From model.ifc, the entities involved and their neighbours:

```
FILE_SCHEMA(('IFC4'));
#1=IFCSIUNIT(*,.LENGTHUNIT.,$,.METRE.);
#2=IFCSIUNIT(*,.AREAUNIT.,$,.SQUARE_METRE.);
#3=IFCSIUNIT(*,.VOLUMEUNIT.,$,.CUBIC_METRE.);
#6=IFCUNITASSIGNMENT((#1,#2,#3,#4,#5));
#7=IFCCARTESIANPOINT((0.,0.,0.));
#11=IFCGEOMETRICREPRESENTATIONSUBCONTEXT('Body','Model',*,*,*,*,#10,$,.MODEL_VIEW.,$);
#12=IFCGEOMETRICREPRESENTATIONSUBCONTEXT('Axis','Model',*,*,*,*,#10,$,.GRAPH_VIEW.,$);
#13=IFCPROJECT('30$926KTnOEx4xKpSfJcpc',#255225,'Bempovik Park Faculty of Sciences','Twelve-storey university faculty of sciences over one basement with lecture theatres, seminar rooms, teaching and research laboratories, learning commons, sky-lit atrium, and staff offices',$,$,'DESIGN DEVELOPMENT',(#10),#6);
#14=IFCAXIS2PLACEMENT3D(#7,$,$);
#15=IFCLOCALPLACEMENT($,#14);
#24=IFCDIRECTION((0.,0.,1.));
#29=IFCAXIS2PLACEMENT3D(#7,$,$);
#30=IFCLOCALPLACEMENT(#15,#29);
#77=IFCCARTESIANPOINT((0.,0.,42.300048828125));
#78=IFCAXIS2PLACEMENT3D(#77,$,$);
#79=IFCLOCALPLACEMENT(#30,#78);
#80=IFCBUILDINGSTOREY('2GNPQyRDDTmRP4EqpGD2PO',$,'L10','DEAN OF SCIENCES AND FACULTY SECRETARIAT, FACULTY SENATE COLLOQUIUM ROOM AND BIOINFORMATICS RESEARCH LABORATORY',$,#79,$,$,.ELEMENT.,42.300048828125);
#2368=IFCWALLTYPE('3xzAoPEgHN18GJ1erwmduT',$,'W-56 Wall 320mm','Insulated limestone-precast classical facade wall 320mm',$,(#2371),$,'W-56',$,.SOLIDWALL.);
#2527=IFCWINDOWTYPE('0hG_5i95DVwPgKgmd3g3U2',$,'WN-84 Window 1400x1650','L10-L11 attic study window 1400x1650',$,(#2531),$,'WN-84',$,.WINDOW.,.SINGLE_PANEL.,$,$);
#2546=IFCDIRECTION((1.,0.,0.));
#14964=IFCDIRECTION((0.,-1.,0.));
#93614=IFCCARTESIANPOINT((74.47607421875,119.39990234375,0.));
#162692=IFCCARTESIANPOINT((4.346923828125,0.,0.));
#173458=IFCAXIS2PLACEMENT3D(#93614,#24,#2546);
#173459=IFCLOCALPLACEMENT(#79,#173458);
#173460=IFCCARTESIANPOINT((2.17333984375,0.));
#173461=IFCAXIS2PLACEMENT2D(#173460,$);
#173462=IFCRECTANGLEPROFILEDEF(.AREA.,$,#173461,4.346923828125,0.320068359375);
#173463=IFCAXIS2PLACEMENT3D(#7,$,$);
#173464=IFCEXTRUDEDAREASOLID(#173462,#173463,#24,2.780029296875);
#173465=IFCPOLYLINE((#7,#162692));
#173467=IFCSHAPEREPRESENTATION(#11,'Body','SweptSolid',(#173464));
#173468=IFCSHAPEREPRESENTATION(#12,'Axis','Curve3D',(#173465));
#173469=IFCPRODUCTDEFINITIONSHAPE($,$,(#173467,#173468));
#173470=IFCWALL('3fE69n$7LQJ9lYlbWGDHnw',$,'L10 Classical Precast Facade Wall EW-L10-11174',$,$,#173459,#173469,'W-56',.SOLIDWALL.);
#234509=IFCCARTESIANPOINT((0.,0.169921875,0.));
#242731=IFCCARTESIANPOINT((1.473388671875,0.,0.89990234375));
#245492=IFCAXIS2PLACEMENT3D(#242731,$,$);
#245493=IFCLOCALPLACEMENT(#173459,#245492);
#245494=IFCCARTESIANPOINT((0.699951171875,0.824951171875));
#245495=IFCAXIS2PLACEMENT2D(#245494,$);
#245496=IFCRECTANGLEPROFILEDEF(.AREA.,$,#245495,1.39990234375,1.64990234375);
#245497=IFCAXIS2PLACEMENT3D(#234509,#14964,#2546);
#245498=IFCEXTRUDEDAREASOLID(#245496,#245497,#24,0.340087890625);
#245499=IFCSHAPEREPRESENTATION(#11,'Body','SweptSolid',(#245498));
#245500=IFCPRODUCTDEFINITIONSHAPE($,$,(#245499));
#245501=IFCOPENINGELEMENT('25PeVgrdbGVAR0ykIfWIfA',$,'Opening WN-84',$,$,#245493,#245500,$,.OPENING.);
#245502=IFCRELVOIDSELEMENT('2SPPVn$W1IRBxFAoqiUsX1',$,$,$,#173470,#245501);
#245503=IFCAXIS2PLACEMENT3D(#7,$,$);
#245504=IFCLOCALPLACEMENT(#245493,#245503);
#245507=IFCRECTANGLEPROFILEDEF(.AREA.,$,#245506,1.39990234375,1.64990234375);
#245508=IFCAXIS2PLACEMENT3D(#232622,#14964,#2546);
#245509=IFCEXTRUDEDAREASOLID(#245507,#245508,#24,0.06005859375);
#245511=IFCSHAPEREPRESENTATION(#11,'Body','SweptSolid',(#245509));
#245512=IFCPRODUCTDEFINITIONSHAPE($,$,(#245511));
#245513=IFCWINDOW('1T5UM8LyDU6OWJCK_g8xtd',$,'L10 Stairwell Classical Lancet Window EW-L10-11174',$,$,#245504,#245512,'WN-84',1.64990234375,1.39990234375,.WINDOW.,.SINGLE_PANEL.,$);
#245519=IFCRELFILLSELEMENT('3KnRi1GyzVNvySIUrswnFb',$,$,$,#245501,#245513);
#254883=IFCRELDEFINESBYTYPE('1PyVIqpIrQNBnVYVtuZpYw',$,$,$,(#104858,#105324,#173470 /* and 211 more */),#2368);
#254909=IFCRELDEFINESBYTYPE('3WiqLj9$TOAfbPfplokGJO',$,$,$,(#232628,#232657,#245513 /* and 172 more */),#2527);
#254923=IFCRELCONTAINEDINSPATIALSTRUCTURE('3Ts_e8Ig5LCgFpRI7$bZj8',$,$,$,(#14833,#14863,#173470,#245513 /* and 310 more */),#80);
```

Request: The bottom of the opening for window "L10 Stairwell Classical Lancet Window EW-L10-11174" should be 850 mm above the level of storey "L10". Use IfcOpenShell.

```python
import numpy as np
import ifcopenshell
import ifcopenshell.api.geometry
import ifcopenshell.geom
import ifcopenshell.util.element
import ifcopenshell.util.placement
import ifcopenshell.util.shape
import ifcopenshell.util.unit

model = ifcopenshell.open("model.ifc")
unit_scale = ifcopenshell.util.unit.calculate_unit_scale(model)

window = model.by_id(245513)
opening = window.FillsVoids[0].RelatingOpeningElement
storey = ifcopenshell.util.element.get_container(window, ifc_class="IfcBuildingStorey")
level = ifcopenshell.util.placement.get_local_placement(storey.ObjectPlacement)[2, 3]

# The opening's origin need not be at the sill, so measure its lowest point.
shape = ifcopenshell.geom.create_shape(ifcopenshell.geom.settings(), opening)
bottom = ifcopenshell.util.shape.get_shape_bottom_elevation(shape, shape.geometry) / unit_scale
dz = level + 0.85 / unit_scale - bottom

shift = np.array([0.0, 0.0, dz])
# The window is placed relative to its opening, so it follows when the opening moves.
matrix = ifcopenshell.util.placement.get_local_placement(opening.ObjectPlacement)
matrix[:3, 3] += shift
ifcopenshell.api.geometry.edit_object_placement(
    model, product=opening, matrix=matrix, is_si=False, should_transform_children=True
)

print(f"moved by {dz * unit_scale:+.3f} m")

model.write("model_v2.ifc")
```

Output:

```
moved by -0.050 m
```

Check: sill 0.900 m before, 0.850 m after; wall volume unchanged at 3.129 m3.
